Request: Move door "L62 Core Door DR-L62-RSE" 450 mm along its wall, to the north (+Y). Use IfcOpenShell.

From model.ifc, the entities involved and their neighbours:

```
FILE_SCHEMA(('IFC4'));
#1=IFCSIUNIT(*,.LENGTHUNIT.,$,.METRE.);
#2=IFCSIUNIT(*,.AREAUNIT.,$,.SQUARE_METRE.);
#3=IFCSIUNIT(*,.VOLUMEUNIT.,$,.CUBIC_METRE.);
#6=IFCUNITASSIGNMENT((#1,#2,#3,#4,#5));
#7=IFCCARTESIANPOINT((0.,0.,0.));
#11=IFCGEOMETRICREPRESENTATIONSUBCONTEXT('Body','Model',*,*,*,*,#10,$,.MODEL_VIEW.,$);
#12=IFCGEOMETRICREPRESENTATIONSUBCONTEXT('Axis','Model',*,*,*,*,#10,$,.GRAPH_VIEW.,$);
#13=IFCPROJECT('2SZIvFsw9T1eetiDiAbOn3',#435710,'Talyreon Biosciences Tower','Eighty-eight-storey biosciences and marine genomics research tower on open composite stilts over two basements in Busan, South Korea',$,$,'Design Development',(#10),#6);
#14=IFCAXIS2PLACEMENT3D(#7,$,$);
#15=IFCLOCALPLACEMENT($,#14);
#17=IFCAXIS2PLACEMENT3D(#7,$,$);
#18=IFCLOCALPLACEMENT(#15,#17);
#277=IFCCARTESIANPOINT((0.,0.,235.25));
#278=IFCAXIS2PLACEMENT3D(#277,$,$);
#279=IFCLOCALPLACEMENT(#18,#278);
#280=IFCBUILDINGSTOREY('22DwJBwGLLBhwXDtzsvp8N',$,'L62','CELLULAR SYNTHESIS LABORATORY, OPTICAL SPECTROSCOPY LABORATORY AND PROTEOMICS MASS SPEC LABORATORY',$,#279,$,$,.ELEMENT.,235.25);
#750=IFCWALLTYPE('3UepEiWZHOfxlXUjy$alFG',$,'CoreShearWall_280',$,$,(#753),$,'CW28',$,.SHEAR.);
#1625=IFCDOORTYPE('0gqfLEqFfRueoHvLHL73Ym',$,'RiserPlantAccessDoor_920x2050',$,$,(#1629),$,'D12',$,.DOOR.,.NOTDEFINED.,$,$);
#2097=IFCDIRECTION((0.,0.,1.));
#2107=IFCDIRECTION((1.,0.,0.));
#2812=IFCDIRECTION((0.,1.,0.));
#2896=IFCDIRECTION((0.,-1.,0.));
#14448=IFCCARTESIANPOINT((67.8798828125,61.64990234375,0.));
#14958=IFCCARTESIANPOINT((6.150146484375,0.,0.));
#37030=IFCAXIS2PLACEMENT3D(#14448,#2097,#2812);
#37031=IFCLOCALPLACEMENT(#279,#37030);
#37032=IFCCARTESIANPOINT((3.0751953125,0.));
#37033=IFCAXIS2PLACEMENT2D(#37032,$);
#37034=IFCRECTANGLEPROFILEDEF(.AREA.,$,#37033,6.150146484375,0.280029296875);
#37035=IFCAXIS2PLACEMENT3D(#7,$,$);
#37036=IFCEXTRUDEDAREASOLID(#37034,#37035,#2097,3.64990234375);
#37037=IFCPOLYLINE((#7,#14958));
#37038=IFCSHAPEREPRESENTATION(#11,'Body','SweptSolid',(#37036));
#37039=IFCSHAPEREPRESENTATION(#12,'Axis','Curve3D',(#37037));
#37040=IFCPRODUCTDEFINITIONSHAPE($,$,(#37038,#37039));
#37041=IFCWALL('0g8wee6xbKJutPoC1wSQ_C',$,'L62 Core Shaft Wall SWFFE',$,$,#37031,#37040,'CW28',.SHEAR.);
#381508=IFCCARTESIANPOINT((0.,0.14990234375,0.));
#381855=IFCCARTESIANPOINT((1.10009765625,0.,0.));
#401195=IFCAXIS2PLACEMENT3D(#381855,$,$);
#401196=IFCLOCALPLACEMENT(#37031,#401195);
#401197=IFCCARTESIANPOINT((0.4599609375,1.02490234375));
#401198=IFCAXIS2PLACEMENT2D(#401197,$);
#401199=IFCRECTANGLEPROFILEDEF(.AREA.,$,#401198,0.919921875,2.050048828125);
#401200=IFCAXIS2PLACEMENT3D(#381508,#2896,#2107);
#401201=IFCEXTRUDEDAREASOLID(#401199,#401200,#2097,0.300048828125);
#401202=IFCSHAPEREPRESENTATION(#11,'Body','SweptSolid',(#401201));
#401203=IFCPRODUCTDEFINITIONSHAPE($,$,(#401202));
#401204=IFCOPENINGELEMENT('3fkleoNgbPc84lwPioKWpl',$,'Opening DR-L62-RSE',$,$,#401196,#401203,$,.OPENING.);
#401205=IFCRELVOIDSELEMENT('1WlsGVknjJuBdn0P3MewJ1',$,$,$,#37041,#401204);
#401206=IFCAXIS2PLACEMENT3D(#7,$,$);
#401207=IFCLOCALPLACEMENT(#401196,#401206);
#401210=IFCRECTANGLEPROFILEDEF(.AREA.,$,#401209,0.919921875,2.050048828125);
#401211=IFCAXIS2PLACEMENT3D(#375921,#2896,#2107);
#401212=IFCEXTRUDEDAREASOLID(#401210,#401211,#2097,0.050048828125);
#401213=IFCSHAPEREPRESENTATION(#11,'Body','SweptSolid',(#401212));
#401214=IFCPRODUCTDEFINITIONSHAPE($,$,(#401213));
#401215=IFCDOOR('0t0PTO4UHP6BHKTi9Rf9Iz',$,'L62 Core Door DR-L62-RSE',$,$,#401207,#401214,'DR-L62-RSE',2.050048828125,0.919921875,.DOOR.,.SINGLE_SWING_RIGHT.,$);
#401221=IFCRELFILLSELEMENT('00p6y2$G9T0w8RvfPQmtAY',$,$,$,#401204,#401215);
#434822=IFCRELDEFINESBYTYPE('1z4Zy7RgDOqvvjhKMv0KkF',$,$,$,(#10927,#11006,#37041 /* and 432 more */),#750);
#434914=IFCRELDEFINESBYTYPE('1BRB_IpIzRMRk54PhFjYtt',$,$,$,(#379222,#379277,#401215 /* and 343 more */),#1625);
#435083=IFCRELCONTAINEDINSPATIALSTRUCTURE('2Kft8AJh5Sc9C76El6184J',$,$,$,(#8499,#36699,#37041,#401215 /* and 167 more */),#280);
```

```python
import ifcopenshell
import ifcopenshell.api.geometry
import ifcopenshell.util.placement

model = ifcopenshell.open("model.ifc")

door = model.by_guid("0t0PTO4UHP6BHKTi9Rf9Iz")
opening = door.FillsVoids[0].RelatingOpeningElement
wall = opening.VoidsElements[0].RelatingBuildingElement

wall_matrix = ifcopenshell.util.placement.get_local_placement(wall.ObjectPlacement)
shift = wall_matrix[:3, 0] * 0.45
before = ifcopenshell.util.placement.get_local_placement(door.ObjectPlacement)[:3, 3].copy()

# The door is placed relative to its opening, so it follows when the opening moves.
matrix = ifcopenshell.util.placement.get_local_placement(opening.ObjectPlacement)
matrix[:3, 3] += shift
ifcopenshell.api.geometry.edit_object_placement(
    model, product=opening, matrix=matrix, is_si=False, should_transform_children=True
)

after = ifcopenshell.util.placement.get_local_placement(door.ObjectPlacement)[:3, 3]
print("door moved by", (after - before).round(3) + 0.0)

model.write("model_updated.ifc")
```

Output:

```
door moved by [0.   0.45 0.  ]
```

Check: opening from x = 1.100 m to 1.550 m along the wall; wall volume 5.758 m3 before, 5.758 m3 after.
